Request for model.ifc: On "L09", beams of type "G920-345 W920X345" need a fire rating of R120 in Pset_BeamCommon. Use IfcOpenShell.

First a look at what the model holds.

```python
import ifcopenshell
import ifcopenshell.util.element

model = ifcopenshell.open("model.ifc")
print(model.schema)
storey = next(s for s in model.by_type("IfcBuildingStorey") if s.Name == "L09")
beams = [e for e in ifcopenshell.util.element.get_decomposition(storey) if e.is_a("IfcBeam")]
seen = {}
for e in beams:
    element_type = ifcopenshell.util.element.get_type(e)
    key = (element_type.Name if element_type != e and element_type else None, ifcopenshell.util.element.get_pset(e, "Pset_BeamCommon", "FireRating"))
    seen[key] = seen.get(key, 0) + 1
for (name, value), count in sorted(seen.items(), key=str):
    print(count, "x", name, "|", value)
```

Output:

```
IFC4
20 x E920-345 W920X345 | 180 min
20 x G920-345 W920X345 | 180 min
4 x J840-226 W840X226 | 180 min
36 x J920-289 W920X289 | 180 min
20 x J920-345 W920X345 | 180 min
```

```python
import ifcopenshell
import ifcopenshell.api.pset
import ifcopenshell.util.element

model = ifcopenshell.open("model.ifc")

storey = next(s for s in model.by_type("IfcBuildingStorey") if s.Name == "L09")
beams = [e for e in ifcopenshell.util.element.get_decomposition(storey) if e.is_a("IfcBeam")]

count = 0
for e in beams:
    element_type = ifcopenshell.util.element.get_type(e)
    if element_type in (None, e) or element_type.Name != "G920-345 W920X345":
        continue
    found = ifcopenshell.util.element.get_pset(e, "Pset_BeamCommon", should_inherit=False)
    if found:
        pset = model.by_id(found["id"])
        if len(ifcopenshell.util.element.get_elements_by_pset(pset)) > 1:
            pset = ifcopenshell.api.pset.unshare_pset(model, products=[e], pset=pset)[0]
    else:
        pset = ifcopenshell.api.pset.add_pset(model, product=e, name="Pset_BeamCommon")
    ifcopenshell.api.pset.edit_pset(model, pset=pset, properties={"FireRating": "R120"})
    count += 1

print(count, "beams updated")

model.write("model_v2.ifc")
```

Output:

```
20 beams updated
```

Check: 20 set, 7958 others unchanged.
